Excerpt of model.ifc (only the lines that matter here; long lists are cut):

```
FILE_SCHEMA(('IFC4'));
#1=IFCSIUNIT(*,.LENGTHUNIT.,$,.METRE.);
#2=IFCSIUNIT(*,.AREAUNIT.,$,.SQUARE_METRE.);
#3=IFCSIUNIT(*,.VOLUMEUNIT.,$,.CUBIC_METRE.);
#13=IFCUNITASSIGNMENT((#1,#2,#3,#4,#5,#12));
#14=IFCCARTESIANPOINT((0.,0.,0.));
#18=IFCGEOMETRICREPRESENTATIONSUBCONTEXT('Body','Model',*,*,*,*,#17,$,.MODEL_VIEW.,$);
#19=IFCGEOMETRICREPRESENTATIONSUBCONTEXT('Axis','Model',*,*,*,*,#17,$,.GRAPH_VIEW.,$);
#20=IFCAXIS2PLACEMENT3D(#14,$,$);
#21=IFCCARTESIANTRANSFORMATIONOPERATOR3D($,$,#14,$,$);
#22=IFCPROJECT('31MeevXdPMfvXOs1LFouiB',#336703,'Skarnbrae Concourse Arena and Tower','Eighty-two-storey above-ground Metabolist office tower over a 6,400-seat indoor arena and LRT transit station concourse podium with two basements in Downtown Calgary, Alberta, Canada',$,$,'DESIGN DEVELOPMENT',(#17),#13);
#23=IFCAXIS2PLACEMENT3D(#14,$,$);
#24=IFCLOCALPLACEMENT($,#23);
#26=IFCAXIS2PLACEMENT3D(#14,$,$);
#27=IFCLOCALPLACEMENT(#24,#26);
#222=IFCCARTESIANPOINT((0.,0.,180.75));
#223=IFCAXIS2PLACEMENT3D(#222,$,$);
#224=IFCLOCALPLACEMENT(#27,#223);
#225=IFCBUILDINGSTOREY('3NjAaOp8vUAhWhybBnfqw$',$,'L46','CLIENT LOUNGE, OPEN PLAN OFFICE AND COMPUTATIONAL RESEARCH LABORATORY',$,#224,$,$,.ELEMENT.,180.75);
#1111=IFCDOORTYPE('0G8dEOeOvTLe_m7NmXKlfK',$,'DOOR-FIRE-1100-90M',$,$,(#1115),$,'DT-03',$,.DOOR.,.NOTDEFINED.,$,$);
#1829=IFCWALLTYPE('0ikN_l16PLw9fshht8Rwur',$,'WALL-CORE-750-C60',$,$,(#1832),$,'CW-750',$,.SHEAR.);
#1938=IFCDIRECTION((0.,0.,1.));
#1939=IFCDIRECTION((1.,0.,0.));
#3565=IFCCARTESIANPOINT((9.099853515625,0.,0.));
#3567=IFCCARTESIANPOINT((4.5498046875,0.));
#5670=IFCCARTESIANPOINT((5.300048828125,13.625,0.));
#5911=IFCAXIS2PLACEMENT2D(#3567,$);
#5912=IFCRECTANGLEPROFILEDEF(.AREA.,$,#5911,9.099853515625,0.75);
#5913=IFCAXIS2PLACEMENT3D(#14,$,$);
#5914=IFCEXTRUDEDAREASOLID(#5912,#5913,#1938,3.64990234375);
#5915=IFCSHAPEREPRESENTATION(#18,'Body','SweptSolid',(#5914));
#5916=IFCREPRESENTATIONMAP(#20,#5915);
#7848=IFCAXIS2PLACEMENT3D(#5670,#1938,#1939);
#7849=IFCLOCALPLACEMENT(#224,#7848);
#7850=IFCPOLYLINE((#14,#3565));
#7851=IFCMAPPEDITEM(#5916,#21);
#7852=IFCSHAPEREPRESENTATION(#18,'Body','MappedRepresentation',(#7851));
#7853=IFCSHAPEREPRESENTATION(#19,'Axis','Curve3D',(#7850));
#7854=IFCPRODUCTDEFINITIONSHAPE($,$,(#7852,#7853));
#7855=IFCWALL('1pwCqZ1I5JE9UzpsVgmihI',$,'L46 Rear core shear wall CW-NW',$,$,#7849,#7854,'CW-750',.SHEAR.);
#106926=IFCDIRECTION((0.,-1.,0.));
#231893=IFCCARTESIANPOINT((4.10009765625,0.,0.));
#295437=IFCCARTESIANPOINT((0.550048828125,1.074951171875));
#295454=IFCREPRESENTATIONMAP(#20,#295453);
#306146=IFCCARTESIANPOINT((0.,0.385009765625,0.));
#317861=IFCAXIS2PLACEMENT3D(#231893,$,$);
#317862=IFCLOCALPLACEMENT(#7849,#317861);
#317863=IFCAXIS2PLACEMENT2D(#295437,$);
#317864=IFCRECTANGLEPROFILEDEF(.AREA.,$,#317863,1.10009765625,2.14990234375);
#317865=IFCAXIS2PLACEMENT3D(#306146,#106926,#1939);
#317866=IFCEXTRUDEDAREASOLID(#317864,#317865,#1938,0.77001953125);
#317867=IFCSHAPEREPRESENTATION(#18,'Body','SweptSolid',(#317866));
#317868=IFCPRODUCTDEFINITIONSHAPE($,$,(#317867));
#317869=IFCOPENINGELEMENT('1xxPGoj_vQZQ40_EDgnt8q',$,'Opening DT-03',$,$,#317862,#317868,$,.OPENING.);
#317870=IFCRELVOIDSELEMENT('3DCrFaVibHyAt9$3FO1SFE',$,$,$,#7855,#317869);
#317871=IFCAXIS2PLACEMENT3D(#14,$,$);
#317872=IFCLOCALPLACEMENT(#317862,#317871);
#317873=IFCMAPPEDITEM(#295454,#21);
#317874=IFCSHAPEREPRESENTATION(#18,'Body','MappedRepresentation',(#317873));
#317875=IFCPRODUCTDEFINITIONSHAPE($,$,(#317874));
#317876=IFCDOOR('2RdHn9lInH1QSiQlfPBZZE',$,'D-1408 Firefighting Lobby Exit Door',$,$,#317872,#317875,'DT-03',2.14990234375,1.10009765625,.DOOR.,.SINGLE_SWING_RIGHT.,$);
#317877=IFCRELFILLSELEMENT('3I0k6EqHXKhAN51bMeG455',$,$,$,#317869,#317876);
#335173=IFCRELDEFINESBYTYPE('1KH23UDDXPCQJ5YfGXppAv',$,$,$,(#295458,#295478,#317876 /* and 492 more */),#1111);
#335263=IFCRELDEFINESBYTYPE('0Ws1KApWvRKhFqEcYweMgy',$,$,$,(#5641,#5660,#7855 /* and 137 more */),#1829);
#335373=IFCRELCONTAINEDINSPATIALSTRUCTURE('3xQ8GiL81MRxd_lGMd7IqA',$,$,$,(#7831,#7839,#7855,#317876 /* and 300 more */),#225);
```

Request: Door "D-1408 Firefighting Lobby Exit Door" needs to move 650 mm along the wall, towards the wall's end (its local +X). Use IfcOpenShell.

```python
import ifcopenshell
import ifcopenshell.api.geometry
import ifcopenshell.util.placement

model = ifcopenshell.open("model.ifc")

door = model.by_guid("2RdHn9lInH1QSiQlfPBZZE")
opening = door.FillsVoids[0].RelatingOpeningElement
wall = opening.VoidsElements[0].RelatingBuildingElement

wall_matrix = ifcopenshell.util.placement.get_local_placement(wall.ObjectPlacement)
shift = wall_matrix[:3, 0] * 0.65
before = ifcopenshell.util.placement.get_local_placement(door.ObjectPlacement)[:3, 3].copy()

# The door is placed relative to its opening, so it follows when the opening moves.
matrix = ifcopenshell.util.placement.get_local_placement(opening.ObjectPlacement)
matrix[:3, 3] += shift
ifcopenshell.api.geometry.edit_object_placement(
    model, product=opening, matrix=matrix, is_si=False, should_transform_children=True
)

after = ifcopenshell.util.placement.get_local_placement(door.ObjectPlacement)[:3, 3]
print("door moved by", (after - before).round(3) + 0.0)

model.write("model_edited.ifc")
```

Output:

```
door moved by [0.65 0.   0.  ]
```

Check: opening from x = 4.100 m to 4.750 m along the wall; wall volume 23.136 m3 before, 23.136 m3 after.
